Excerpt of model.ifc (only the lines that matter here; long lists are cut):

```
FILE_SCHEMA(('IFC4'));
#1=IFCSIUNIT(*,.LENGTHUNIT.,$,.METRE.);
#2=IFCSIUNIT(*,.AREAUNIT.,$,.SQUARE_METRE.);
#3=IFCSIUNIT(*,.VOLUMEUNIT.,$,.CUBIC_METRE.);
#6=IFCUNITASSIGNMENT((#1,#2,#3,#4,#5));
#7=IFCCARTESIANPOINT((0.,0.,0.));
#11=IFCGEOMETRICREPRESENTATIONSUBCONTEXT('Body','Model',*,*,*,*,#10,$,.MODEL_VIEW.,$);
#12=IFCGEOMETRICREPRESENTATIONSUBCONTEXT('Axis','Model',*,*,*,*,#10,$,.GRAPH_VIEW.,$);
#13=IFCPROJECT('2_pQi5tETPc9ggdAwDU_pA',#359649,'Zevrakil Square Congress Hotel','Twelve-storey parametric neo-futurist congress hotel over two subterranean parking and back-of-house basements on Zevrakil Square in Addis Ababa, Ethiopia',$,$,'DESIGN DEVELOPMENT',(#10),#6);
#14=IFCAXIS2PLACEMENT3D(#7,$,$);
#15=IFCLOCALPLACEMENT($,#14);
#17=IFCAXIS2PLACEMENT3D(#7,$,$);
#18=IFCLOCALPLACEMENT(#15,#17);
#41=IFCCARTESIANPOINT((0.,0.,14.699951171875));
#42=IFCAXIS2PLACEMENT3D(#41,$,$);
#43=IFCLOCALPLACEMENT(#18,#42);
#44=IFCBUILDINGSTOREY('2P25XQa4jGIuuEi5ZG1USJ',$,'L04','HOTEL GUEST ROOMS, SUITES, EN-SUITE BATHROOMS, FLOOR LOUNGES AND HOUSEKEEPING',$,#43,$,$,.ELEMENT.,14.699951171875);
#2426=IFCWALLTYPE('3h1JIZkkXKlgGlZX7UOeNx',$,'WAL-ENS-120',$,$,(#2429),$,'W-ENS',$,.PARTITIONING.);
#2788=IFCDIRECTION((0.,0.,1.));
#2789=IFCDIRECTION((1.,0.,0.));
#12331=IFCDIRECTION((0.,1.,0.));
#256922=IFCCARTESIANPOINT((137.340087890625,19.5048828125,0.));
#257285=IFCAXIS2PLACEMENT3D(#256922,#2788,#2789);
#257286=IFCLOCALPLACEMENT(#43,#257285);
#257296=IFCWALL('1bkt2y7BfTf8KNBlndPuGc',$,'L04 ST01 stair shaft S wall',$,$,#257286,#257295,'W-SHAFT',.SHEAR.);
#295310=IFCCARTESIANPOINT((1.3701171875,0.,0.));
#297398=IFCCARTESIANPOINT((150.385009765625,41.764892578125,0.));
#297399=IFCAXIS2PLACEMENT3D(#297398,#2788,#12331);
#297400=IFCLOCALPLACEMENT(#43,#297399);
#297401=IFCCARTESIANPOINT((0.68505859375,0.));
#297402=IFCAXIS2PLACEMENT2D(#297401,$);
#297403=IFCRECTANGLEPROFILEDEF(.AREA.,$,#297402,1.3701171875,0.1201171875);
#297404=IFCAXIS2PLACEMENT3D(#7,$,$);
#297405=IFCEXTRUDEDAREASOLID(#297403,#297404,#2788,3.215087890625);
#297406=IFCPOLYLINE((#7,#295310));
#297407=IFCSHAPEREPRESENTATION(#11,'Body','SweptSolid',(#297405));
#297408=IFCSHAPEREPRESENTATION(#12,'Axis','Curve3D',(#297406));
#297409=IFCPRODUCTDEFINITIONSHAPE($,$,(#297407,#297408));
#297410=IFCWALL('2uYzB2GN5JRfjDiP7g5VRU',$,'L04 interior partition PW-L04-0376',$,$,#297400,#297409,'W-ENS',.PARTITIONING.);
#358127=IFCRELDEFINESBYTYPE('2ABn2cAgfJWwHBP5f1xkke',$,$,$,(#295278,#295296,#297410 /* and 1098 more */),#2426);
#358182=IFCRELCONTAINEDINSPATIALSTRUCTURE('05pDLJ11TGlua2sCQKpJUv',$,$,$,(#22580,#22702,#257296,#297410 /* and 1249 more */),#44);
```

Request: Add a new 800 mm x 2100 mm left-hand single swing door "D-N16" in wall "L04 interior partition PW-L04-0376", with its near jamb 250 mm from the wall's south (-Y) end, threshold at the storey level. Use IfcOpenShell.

```python
import numpy as np
import ifcopenshell
import ifcopenshell.api.feature
import ifcopenshell.api.geometry
import ifcopenshell.api.root
import ifcopenshell.api.spatial
import ifcopenshell.geom
import ifcopenshell.util.element
import ifcopenshell.util.placement
import ifcopenshell.util.representation
import ifcopenshell.util.shape
import ifcopenshell.util.unit

model = ifcopenshell.open("model.ifc")
unit_scale = ifcopenshell.util.unit.calculate_unit_scale(model)
settings = ifcopenshell.geom.settings()


def volume(element):
    """Net volume in cubic metres, openings subtracted."""
    shape = ifcopenshell.geom.create_shape(settings, element)
    return ifcopenshell.util.shape.get_volume(shape.geometry)


wall = model.by_guid("2uYzB2GN5JRfjDiP7g5VRU")
storey = ifcopenshell.util.element.get_container(wall, ifc_class="IfcBuildingStorey")
context = ifcopenshell.util.representation.get_context(model, "Model", "Body", "MODEL_VIEW")
before = volume(wall)

width, height, from_end, sill = 0.8, 2.1, 0.25, 0.0  # metres

# The wall runs along its own X axis, and the end named is its -X end.
wall_shape = ifcopenshell.geom.create_shape(settings, wall)
x, y, z = ifcopenshell.util.shape.get_vertices(wall_shape.geometry).T
start = x.min() + from_end
face, thickness = float(y.min()), float(y.max() - y.min())
wall_matrix = ifcopenshell.util.placement.get_local_placement(wall.ObjectPlacement)
level = ifcopenshell.util.placement.get_local_placement(storey.ObjectPlacement)[2, 3]


def in_wall(x, y):
    """Placement at x, y metres in the wall's axes, at sill height."""
    matrix = wall_matrix.copy()
    matrix[:, 3] = wall_matrix @ np.array([x / unit_scale, y / unit_scale, 0.0, 1.0])
    matrix[2, 3] = level + sill / unit_scale
    return matrix


# Opening: a box that overshoots both wall faces by 50 mm.
opening = ifcopenshell.api.root.create_entity(model, ifc_class="IfcOpeningElement", predefined_type="OPENING")
box = ifcopenshell.api.geometry.add_wall_representation(
    model, context=context, length=width, height=height, thickness=thickness + 0.1
)
ifcopenshell.api.geometry.assign_representation(model, product=opening, representation=box)
ifcopenshell.api.geometry.edit_object_placement(model, product=opening, matrix=in_wall(start, face - 0.05), is_si=False)
ifcopenshell.api.feature.add_feature(model, feature=opening, element=wall)

door = ifcopenshell.api.root.create_entity(model, ifc_class="IfcDoor", name="D-N16", predefined_type="DOOR")
door.OverallWidth, door.OverallHeight = width / unit_scale, height / unit_scale
door.OperationType = "SINGLE_SWING_LEFT"
body = ifcopenshell.api.geometry.add_door_representation(
    model,
    context=context,
    overall_width=door.OverallWidth,
    overall_height=door.OverallHeight,
    operation_type="SINGLE_SWING_LEFT",
    lining_properties={"LiningDepth": thickness / unit_scale, "ThresholdDepth": thickness / unit_scale},
)
ifcopenshell.api.geometry.assign_representation(model, product=door, representation=body)
ifcopenshell.api.spatial.assign_container(model, products=[door], relating_structure=storey)
ifcopenshell.api.feature.add_filling(model, opening=opening, element=door)

# The lining spans the wall, so the door starts at the wall face.
ifcopenshell.api.geometry.edit_object_placement(model, product=door, matrix=in_wall(start, face), is_si=False)

after = volume(wall)

print(f"wall volume {before:.3f} -> {after:.3f} m3")

model.write("model_updated.ifc")
```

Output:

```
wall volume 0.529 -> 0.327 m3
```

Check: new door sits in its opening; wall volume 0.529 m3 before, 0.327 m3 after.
